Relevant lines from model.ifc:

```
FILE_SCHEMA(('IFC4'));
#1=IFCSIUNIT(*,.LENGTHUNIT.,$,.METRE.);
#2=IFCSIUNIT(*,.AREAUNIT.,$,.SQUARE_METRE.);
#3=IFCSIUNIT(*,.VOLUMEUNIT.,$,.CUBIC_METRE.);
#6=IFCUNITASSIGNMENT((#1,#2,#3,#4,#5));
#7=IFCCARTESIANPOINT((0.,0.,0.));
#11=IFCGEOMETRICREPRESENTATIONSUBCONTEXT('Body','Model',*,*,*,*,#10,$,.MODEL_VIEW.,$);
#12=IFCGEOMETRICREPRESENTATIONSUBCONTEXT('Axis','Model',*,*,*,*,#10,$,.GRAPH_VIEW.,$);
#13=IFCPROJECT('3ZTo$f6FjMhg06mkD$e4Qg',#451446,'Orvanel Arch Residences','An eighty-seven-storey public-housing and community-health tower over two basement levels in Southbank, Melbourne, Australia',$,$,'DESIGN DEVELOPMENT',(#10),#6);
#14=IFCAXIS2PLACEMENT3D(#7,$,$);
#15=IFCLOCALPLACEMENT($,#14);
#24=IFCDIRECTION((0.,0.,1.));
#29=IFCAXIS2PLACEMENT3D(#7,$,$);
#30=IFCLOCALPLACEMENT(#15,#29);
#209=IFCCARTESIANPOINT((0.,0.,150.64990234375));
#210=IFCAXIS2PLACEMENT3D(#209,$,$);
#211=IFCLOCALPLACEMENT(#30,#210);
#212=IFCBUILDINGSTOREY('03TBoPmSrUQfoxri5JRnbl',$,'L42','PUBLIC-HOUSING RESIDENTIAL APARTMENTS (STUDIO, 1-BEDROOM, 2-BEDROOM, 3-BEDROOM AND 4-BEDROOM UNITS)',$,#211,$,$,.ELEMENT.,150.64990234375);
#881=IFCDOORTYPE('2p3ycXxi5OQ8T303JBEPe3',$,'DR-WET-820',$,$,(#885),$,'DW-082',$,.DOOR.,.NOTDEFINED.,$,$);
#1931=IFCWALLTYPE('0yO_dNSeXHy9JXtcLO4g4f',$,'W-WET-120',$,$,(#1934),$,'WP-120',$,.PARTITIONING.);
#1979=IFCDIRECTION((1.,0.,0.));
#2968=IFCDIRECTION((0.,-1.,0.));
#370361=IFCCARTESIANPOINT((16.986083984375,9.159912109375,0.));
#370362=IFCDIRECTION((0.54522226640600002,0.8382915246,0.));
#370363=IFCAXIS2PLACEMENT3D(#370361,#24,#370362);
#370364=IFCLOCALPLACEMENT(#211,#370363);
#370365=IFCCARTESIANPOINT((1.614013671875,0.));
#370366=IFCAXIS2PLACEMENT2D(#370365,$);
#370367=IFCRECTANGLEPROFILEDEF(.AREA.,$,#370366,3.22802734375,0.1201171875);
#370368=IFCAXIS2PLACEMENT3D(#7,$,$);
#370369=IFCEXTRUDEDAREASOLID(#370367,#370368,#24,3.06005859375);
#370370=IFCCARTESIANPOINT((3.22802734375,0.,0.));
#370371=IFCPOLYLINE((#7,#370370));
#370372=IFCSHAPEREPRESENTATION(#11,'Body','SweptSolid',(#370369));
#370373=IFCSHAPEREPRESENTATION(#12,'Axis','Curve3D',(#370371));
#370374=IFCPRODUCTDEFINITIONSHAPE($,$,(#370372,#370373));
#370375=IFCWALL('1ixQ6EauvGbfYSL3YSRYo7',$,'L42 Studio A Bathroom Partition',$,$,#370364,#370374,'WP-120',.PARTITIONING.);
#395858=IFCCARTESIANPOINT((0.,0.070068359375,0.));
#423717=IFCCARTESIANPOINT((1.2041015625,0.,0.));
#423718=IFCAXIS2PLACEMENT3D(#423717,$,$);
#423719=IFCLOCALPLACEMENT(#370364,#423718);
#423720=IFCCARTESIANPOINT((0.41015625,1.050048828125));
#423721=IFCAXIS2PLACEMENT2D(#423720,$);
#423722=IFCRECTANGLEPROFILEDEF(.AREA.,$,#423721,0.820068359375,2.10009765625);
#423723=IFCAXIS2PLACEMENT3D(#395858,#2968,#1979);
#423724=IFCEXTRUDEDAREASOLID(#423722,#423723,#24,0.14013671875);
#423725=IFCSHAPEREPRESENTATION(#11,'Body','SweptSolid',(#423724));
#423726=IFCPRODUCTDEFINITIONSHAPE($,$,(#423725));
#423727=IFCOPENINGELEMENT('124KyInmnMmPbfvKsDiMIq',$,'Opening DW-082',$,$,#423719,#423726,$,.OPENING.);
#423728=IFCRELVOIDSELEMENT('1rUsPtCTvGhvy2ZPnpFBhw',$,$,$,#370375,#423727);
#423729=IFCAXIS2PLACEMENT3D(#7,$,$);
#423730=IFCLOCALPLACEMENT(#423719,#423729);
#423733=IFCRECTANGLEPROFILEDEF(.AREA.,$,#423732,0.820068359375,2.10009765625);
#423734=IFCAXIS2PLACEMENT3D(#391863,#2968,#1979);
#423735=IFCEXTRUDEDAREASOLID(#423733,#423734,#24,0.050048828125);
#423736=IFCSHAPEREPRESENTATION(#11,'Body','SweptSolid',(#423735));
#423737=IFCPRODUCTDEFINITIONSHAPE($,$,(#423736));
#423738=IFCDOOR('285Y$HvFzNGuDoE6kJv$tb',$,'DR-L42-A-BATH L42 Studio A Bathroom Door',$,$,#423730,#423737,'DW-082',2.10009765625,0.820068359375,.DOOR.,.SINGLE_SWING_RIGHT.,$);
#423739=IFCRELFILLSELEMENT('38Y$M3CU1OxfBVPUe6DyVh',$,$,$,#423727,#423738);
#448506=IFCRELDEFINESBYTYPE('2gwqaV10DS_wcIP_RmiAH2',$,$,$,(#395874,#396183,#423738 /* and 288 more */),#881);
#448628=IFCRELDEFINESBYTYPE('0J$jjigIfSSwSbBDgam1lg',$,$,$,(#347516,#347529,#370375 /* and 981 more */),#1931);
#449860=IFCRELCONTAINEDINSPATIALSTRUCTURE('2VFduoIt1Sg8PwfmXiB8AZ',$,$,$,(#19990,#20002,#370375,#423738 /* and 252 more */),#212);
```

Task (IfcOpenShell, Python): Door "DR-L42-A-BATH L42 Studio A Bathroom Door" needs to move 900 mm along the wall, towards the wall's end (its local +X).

```python
import ifcopenshell
import ifcopenshell.api.geometry
import ifcopenshell.util.placement
import ifcopenshell.util.unit

model = ifcopenshell.open("model.ifc")
unit_scale = ifcopenshell.util.unit.calculate_unit_scale(model)

door = model.by_id(423738)
opening = door.FillsVoids[0].RelatingOpeningElement
wall = opening.VoidsElements[0].RelatingBuildingElement

wall_matrix = ifcopenshell.util.placement.get_local_placement(wall.ObjectPlacement)
shift = wall_matrix[:3, 0] * 0.9 / unit_scale
before = ifcopenshell.util.placement.get_local_placement(door.ObjectPlacement)[:3, 3].copy()

# The door is placed relative to its opening, so it follows when the opening moves.
matrix = ifcopenshell.util.placement.get_local_placement(opening.ObjectPlacement)
matrix[:3, 3] += shift
ifcopenshell.api.geometry.edit_object_placement(
    model, product=opening, matrix=matrix, is_si=False, should_transform_children=True
)

after = ifcopenshell.util.placement.get_local_placement(door.ObjectPlacement)[:3, 3]
print("door moved by", (after - before).round(3) + 0.0)

model.write("model_updated.ifc")
```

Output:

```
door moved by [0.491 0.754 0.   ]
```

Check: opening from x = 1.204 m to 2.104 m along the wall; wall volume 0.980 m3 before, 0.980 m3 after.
